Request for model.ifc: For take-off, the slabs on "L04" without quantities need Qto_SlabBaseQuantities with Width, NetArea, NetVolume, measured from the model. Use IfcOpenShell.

First a look at what the model holds.

```python
import ifcopenshell
import ifcopenshell.util.element
import ifcopenshell.util.unit

model = ifcopenshell.open("model.ifc")
print(model.schema)
for unit_type in ("LENGTHUNIT", "AREAUNIT", "VOLUMEUNIT"):
    print(unit_type, ifcopenshell.util.unit.calculate_unit_scale(model, unit_type))
storey = next(s for s in model.by_type("IfcBuildingStorey") if s.Name == "L04")
slabs = [e for e in ifcopenshell.util.element.get_decomposition(storey) if e.is_a("IfcSlab")]
for e in sorted(slabs, key=lambda e: e.id()):
    print(e.id(), e.is_a(), e.Name, list(ifcopenshell.util.element.get_psets(e, qtos_only=True)), sep=" | ")
```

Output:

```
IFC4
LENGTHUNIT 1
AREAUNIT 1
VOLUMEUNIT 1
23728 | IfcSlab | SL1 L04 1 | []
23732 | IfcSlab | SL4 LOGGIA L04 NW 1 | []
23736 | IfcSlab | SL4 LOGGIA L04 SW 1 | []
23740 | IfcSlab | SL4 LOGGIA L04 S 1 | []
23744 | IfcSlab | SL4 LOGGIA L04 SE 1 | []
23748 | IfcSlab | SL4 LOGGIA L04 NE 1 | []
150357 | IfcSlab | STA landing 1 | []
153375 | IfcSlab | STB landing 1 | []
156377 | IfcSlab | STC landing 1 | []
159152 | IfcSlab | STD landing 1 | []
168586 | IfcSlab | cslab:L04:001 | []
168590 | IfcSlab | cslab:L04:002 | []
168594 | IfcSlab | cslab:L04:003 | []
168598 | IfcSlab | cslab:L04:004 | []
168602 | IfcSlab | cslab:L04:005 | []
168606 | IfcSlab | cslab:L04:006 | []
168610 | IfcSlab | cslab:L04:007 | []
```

```python
import ifcopenshell
import ifcopenshell.api.pset
import ifcopenshell.geom
import ifcopenshell.util.element
import ifcopenshell.util.shape
import ifcopenshell.util.unit

model = ifcopenshell.open("model.ifc")
unit_scale = ifcopenshell.util.unit.calculate_unit_scale(model)
area_scale = ifcopenshell.util.unit.calculate_unit_scale(model, "AREAUNIT")
volume_scale = ifcopenshell.util.unit.calculate_unit_scale(model, "VOLUMEUNIT")
settings = ifcopenshell.geom.settings()

storey = next(s for s in model.by_type("IfcBuildingStorey") if s.Name == "L04")
slabs = [e for e in ifcopenshell.util.element.get_decomposition(storey) if e.is_a("IfcSlab")]

for e in sorted(slabs, key=lambda e: e.id()):
    if ifcopenshell.util.element.get_psets(e, qtos_only=True, should_inherit=False):
        continue
    # Geometry comes back in metres, in the element's own axes.
    shape = ifcopenshell.geom.create_shape(settings, e)
    values = {
        "Width": ifcopenshell.util.shape.get_z(shape.geometry) / unit_scale,
        "NetArea": ifcopenshell.util.shape.get_footprint_area(shape.geometry) / area_scale,
        "NetVolume": ifcopenshell.util.shape.get_volume(shape.geometry) / volume_scale,
    }
    qto = ifcopenshell.api.pset.add_qto(model, product=e, name="Qto_SlabBaseQuantities")
    ifcopenshell.api.pset.edit_qto(model, qto=qto, properties=values)
    print(e.id(), {k: round(v, 3) for k, v in values.items()})

model.write("model_edited.ifc")
```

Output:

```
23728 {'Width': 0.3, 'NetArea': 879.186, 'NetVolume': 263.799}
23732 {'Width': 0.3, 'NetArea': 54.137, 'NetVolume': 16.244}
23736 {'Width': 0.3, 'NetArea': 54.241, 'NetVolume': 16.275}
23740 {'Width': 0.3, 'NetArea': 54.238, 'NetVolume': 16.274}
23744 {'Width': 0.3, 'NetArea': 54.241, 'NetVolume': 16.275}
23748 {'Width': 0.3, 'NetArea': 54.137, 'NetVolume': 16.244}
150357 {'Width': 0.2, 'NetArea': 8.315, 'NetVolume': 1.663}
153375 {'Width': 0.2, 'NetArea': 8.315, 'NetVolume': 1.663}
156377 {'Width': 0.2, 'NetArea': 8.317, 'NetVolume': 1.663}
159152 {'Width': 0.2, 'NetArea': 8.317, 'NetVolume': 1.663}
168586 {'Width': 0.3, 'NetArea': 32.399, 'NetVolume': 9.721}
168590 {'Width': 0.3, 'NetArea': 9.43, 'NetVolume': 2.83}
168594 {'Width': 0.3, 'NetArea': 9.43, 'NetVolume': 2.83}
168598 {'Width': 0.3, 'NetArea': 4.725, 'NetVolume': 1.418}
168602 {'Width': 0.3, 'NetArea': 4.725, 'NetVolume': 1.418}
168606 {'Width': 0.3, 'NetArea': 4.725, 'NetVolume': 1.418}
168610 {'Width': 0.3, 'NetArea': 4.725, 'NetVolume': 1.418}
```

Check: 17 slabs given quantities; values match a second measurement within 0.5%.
